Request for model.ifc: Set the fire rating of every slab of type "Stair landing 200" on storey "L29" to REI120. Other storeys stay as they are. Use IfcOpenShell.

First a look at what the model holds.

```python
import ifcopenshell
import ifcopenshell.util.element

model = ifcopenshell.open("model.ifc")
print(model.schema)
storey = next(s for s in model.by_type("IfcBuildingStorey") if s.Name == "L29")
slabs = [e for e in ifcopenshell.util.element.get_decomposition(storey) if e.is_a("IfcSlab")]
seen = {}
for e in slabs:
    element_type = ifcopenshell.util.element.get_type(e)
    key = (element_type.Name if element_type != e and element_type else None, ifcopenshell.util.element.get_pset(e, "Pset_SlabCommon", "FireRating"))
    seen[key] = seen.get(key, 0) + 1
for (name, value), count in sorted(seen.items(), key=str):
    print(count, "x", name, "|", value)
```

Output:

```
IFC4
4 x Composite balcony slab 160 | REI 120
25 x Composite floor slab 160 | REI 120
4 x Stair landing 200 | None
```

```python
import ifcopenshell
import ifcopenshell.api.pset
import ifcopenshell.util.element

model = ifcopenshell.open("model.ifc")

storey = next(s for s in model.by_type("IfcBuildingStorey") if s.Name == "L29")
slabs = [e for e in ifcopenshell.util.element.get_decomposition(storey) if e.is_a("IfcSlab")]

count = 0
for e in slabs:
    element_type = ifcopenshell.util.element.get_type(e)
    if element_type in (None, e) or element_type.Name != "Stair landing 200":
        continue
    found = ifcopenshell.util.element.get_pset(e, "Pset_SlabCommon", should_inherit=False)
    if found:
        pset = model.by_id(found["id"])
        if len(ifcopenshell.util.element.get_elements_by_pset(pset)) > 1:
            pset = ifcopenshell.api.pset.unshare_pset(model, products=[e], pset=pset)[0]
    else:
        pset = ifcopenshell.api.pset.add_pset(model, product=e, name="Pset_SlabCommon")
    ifcopenshell.api.pset.edit_pset(model, pset=pset, properties={"FireRating": "REI120"})
    count += 1

print(count, "slabs updated")

model.write("model_updated.ifc")
```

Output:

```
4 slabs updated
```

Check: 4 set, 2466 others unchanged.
